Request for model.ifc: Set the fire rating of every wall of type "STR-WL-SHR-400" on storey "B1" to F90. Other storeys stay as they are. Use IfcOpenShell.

First a look at what the model holds.

```python
import ifcopenshell
import ifcopenshell.util.element

model = ifcopenshell.open("model.ifc")
print(model.schema)
storey = next(s for s in model.by_type("IfcBuildingStorey") if s.Name == "B1")
walls = [e for e in ifcopenshell.util.element.get_decomposition(storey) if e.is_a("IfcWall")]
seen = {}
for e in walls:
    element_type = ifcopenshell.util.element.get_type(e)
    key = (element_type.Name if element_type != e and element_type else None, ifcopenshell.util.element.get_pset(e, "Pset_WallCommon", "FireRating"))
    seen[key] = seen.get(key, 0) + 1
for (name, value), count in sorted(seen.items(), key=str):
    print(count, "x", name, "|", value)
```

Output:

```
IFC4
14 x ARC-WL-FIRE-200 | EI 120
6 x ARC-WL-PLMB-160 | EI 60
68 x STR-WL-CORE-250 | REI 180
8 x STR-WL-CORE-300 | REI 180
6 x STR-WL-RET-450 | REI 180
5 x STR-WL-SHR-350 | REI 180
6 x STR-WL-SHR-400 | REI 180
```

```python
import ifcopenshell
import ifcopenshell.api.pset
import ifcopenshell.util.element

model = ifcopenshell.open("model.ifc")

storey = next(s for s in model.by_type("IfcBuildingStorey") if s.Name == "B1")
walls = [e for e in ifcopenshell.util.element.get_decomposition(storey) if e.is_a("IfcWall")]

count = 0
for e in walls:
    element_type = ifcopenshell.util.element.get_type(e)
    if element_type in (None, e) or element_type.Name != "STR-WL-SHR-400":
        continue
    # add_pset returns the element's existing set when there is one.
    pset = ifcopenshell.api.pset.add_pset(model, product=e, name="Pset_WallCommon")
    ifcopenshell.api.pset.edit_pset(model, pset=pset, properties={"FireRating": "F90"})
    count += 1

print(count, "walls updated")

model.write("model_v2.ifc")
```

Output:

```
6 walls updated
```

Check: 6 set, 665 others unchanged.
